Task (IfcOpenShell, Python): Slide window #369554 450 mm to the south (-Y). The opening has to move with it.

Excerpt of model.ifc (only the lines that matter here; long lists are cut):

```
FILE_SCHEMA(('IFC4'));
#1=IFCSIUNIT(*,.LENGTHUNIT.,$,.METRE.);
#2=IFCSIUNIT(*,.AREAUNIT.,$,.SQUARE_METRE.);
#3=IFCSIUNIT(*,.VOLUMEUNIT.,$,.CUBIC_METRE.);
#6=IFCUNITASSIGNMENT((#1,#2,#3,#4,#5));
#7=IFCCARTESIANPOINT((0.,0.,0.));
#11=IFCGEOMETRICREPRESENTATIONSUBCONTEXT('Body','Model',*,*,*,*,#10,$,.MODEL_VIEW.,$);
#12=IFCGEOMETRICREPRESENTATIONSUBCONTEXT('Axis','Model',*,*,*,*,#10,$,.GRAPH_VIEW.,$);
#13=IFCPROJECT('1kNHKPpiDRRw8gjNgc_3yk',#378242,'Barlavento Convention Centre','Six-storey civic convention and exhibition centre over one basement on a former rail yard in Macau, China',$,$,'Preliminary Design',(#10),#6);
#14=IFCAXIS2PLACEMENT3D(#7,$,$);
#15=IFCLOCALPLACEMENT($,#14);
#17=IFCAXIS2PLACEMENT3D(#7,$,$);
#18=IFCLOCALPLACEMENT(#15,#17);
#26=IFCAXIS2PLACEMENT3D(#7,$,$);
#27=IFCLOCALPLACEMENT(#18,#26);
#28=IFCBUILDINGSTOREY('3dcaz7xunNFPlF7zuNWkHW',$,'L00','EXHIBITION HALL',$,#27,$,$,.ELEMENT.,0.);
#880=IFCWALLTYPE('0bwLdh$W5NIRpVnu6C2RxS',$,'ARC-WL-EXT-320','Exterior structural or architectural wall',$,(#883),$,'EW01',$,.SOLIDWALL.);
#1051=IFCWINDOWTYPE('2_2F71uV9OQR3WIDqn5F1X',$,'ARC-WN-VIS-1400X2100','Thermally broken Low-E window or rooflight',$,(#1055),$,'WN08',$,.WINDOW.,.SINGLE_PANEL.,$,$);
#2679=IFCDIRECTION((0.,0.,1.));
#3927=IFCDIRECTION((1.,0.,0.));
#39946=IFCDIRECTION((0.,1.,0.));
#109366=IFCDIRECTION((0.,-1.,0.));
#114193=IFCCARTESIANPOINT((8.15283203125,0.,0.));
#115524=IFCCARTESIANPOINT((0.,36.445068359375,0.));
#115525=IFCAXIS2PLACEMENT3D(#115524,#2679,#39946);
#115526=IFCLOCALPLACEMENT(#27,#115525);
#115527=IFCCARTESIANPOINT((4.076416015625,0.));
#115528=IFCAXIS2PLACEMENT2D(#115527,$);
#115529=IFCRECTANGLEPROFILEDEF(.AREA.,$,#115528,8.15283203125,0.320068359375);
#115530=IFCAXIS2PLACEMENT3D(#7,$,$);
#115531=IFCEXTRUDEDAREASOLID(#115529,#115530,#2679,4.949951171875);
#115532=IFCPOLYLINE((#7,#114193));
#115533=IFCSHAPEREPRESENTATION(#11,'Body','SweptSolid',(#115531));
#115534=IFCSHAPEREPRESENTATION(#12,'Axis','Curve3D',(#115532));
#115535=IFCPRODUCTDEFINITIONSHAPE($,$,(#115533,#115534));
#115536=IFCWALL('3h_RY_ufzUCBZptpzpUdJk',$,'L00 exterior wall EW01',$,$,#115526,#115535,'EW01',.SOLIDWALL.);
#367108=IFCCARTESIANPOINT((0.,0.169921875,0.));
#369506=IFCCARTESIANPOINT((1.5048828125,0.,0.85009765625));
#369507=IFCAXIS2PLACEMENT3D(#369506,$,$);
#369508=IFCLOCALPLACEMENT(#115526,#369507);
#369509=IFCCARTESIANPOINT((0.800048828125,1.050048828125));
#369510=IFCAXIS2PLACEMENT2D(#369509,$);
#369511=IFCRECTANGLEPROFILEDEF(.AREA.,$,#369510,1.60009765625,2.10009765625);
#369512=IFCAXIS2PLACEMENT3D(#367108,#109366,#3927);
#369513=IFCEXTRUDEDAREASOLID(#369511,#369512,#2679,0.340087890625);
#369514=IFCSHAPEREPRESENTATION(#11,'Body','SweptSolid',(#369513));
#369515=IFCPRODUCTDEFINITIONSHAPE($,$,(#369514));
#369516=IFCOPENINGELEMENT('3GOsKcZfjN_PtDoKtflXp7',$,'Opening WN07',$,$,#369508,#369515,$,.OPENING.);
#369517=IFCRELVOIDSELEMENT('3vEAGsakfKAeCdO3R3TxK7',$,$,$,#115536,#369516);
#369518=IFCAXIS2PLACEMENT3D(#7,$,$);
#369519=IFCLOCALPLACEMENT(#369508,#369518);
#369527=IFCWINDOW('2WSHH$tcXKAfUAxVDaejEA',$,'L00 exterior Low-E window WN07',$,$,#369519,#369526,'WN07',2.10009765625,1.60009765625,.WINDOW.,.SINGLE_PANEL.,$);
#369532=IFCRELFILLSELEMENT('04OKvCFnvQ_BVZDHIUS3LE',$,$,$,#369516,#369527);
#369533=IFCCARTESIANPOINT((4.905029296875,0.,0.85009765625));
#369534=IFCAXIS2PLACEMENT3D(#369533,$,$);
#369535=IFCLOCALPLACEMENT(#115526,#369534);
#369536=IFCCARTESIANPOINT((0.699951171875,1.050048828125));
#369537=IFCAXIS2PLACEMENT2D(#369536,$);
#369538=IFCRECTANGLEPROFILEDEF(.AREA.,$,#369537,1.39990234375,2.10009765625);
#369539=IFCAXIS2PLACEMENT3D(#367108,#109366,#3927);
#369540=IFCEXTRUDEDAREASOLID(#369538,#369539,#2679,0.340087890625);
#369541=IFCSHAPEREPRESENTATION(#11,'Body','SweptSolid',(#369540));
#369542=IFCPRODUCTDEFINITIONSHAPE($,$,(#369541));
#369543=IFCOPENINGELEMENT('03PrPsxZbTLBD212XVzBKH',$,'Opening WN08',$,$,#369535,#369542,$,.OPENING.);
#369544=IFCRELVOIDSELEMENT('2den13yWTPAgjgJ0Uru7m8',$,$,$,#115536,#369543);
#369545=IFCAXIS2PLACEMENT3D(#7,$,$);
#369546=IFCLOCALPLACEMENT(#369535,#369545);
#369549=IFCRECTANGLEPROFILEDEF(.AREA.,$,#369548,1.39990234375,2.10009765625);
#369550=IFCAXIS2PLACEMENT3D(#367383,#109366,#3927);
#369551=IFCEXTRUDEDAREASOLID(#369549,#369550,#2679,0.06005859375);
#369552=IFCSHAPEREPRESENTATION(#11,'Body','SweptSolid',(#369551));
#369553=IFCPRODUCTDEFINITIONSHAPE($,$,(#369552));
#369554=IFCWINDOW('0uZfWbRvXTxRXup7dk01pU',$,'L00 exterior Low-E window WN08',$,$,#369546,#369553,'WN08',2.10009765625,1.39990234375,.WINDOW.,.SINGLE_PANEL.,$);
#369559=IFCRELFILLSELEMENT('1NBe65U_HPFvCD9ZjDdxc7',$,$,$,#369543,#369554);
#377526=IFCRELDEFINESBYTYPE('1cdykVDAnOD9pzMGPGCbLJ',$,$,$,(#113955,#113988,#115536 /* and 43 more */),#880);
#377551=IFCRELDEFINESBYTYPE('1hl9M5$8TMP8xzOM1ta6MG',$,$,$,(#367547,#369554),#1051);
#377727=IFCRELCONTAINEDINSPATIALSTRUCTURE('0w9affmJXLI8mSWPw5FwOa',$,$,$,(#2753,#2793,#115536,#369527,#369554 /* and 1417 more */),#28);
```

```python
import ifcopenshell
import ifcopenshell.api.geometry
import ifcopenshell.util.placement

model = ifcopenshell.open("model.ifc")

window = model.by_guid("0uZfWbRvXTxRXup7dk01pU")
opening = window.FillsVoids[0].RelatingOpeningElement
wall = opening.VoidsElements[0].RelatingBuildingElement

wall_matrix = ifcopenshell.util.placement.get_local_placement(wall.ObjectPlacement)
shift = wall_matrix[:3, 0] * -0.45
before = ifcopenshell.util.placement.get_local_placement(window.ObjectPlacement)[:3, 3].copy()

# The window is placed relative to its opening, so it follows when the opening moves.
matrix = ifcopenshell.util.placement.get_local_placement(opening.ObjectPlacement)
matrix[:3, 3] += shift
ifcopenshell.api.geometry.edit_object_placement(
    model, product=opening, matrix=matrix, is_si=False, should_transform_children=True
)

after = ifcopenshell.util.placement.get_local_placement(window.ObjectPlacement)[:3, 3]
print("window moved by", (after - before).round(3) + 0.0)

model.write("model_edited.ifc")
```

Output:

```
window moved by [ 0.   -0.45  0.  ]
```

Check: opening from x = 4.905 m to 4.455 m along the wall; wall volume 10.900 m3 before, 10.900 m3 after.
